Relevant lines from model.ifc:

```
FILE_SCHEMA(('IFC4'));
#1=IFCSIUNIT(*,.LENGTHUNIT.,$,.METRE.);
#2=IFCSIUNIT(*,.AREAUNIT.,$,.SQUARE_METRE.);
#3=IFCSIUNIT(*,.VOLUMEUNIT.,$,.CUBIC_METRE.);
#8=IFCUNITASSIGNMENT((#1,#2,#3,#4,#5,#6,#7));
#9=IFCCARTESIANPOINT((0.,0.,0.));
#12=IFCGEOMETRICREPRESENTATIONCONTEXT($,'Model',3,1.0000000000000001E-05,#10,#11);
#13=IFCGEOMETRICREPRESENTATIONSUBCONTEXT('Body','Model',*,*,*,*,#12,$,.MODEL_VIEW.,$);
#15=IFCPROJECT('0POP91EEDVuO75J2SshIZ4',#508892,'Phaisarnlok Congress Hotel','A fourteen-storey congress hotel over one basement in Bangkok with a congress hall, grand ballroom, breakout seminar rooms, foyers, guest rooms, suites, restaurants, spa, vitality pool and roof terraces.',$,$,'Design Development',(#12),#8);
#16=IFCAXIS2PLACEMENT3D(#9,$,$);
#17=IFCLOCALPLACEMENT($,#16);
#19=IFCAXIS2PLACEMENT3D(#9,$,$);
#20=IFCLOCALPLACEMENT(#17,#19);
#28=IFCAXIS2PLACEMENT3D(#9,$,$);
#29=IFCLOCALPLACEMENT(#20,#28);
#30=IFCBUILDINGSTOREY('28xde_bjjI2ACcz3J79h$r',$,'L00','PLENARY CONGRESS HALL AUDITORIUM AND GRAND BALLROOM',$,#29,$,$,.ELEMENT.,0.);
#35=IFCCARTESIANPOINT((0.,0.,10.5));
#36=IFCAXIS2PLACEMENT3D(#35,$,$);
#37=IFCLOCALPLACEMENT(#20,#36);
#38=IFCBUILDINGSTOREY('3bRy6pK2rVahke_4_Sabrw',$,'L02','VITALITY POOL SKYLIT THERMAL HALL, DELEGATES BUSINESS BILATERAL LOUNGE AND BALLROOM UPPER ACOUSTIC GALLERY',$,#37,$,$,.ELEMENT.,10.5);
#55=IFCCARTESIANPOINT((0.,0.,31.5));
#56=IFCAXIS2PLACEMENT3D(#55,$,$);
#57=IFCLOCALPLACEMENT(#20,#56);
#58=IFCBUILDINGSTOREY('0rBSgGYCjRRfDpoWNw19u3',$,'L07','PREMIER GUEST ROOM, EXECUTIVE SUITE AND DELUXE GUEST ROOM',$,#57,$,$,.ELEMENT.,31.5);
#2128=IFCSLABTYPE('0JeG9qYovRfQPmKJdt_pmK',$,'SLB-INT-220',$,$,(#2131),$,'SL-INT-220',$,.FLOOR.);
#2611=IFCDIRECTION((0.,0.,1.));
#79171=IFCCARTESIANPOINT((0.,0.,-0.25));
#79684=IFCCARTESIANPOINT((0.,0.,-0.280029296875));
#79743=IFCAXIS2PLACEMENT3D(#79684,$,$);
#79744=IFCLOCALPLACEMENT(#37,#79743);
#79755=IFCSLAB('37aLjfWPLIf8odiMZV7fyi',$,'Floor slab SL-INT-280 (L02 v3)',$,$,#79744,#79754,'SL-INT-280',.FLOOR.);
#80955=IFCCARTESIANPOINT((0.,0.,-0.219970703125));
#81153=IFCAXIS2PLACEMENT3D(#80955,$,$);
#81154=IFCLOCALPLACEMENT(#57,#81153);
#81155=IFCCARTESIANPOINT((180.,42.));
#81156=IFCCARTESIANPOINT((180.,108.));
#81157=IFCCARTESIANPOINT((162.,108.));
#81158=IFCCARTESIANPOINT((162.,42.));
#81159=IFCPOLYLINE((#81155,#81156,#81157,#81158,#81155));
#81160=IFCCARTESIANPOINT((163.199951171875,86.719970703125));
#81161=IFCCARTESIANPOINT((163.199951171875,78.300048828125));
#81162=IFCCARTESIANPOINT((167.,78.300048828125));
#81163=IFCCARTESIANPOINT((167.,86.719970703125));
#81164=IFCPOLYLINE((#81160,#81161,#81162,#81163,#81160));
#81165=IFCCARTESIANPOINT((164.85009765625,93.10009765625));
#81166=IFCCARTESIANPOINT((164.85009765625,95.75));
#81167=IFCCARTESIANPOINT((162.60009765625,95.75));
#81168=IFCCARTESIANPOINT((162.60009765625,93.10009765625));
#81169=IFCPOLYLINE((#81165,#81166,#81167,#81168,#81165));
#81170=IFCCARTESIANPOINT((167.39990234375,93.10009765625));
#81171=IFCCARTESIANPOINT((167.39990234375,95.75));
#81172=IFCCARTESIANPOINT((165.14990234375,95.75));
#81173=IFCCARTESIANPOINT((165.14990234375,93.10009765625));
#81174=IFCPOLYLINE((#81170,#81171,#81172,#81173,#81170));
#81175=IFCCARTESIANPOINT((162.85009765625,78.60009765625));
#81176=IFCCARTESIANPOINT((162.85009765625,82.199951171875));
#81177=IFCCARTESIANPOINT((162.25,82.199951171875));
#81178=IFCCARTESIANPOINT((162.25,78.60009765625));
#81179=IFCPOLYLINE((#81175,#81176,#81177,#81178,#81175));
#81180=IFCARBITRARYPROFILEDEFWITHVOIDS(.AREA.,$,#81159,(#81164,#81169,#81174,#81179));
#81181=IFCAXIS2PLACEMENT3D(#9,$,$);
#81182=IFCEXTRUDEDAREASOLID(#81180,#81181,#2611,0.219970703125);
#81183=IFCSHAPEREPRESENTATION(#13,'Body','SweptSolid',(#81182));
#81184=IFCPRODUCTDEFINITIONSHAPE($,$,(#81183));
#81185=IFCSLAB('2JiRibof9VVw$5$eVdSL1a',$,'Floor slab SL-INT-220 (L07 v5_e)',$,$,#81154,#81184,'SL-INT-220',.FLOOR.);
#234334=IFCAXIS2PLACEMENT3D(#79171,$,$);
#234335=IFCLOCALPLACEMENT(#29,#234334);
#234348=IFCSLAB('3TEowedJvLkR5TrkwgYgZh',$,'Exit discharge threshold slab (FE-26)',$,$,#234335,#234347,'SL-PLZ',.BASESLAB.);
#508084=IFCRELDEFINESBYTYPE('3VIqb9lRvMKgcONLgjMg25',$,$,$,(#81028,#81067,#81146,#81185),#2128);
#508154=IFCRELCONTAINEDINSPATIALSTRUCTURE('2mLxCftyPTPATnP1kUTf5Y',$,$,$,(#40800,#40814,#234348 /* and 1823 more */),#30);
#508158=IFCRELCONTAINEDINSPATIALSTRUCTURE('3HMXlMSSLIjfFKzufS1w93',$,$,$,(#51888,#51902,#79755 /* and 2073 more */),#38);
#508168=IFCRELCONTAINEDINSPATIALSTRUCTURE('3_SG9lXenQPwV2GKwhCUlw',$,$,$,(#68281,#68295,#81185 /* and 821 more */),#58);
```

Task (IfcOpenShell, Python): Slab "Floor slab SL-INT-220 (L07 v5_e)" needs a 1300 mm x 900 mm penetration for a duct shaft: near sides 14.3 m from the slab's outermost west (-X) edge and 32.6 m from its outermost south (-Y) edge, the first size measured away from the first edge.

```python
import numpy as np
import ifcopenshell
import ifcopenshell.api.feature
import ifcopenshell.api.geometry
import ifcopenshell.api.root
import ifcopenshell.geom
import ifcopenshell.util.placement
import ifcopenshell.util.representation
import ifcopenshell.util.shape
import ifcopenshell.util.unit

model = ifcopenshell.open("model.ifc")
unit_scale = ifcopenshell.util.unit.calculate_unit_scale(model)
settings = ifcopenshell.geom.settings()


def volume(element):
    """Net volume in cubic metres, openings subtracted."""
    shape = ifcopenshell.geom.create_shape(settings, element)
    return ifcopenshell.util.shape.get_volume(shape.geometry)


slab = model.by_guid("2JiRibof9VVw$5$eVdSL1a")
before = volume(slab)

# Extent in the slab's own axes, in metres. The edges named are its -X and -Y sides.
slab_shape = ifcopenshell.geom.create_shape(settings, slab)
vertices = ifcopenshell.util.shape.get_vertices(slab_shape.geometry)
x_min, y_min, bottom = vertices.min(axis=0)
top = vertices[:, 2].max()

opening = ifcopenshell.api.root.create_entity(model, ifc_class="IfcOpeningElement", name="Duct shaft opening", predefined_type="OPENING")
context = ifcopenshell.util.representation.get_context(model, "Model", "Body", "MODEL_VIEW")
width, depth = 1.3, 0.9
outline = [(0.0, 0.0), (width, 0.0), (width, depth), (0.0, depth), (0.0, 0.0)]
# Overshoot both faces by 50 mm so the cut is clean.
shape = ifcopenshell.api.geometry.add_slab_representation(
    model, context=context, depth=top - bottom + 0.1, polyline=outline
)
ifcopenshell.api.geometry.assign_representation(model, product=opening, representation=shape)

matrix = ifcopenshell.util.placement.get_local_placement(slab.ObjectPlacement)
matrix[:, 3] = matrix @ np.append(np.array([x_min + 14.3, y_min + 32.6, bottom - 0.05]) / unit_scale, 1.0)
ifcopenshell.api.geometry.edit_object_placement(model, product=opening, matrix=matrix, is_si=False)
ifcopenshell.api.feature.add_feature(model, feature=opening, element=slab)

after = volume(slab)

print(f"slab volume {before:.3f} -> {after:.3f} m3")

model.write("model_edited.ifc")
```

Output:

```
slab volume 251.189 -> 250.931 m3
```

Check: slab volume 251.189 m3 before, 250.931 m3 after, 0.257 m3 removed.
